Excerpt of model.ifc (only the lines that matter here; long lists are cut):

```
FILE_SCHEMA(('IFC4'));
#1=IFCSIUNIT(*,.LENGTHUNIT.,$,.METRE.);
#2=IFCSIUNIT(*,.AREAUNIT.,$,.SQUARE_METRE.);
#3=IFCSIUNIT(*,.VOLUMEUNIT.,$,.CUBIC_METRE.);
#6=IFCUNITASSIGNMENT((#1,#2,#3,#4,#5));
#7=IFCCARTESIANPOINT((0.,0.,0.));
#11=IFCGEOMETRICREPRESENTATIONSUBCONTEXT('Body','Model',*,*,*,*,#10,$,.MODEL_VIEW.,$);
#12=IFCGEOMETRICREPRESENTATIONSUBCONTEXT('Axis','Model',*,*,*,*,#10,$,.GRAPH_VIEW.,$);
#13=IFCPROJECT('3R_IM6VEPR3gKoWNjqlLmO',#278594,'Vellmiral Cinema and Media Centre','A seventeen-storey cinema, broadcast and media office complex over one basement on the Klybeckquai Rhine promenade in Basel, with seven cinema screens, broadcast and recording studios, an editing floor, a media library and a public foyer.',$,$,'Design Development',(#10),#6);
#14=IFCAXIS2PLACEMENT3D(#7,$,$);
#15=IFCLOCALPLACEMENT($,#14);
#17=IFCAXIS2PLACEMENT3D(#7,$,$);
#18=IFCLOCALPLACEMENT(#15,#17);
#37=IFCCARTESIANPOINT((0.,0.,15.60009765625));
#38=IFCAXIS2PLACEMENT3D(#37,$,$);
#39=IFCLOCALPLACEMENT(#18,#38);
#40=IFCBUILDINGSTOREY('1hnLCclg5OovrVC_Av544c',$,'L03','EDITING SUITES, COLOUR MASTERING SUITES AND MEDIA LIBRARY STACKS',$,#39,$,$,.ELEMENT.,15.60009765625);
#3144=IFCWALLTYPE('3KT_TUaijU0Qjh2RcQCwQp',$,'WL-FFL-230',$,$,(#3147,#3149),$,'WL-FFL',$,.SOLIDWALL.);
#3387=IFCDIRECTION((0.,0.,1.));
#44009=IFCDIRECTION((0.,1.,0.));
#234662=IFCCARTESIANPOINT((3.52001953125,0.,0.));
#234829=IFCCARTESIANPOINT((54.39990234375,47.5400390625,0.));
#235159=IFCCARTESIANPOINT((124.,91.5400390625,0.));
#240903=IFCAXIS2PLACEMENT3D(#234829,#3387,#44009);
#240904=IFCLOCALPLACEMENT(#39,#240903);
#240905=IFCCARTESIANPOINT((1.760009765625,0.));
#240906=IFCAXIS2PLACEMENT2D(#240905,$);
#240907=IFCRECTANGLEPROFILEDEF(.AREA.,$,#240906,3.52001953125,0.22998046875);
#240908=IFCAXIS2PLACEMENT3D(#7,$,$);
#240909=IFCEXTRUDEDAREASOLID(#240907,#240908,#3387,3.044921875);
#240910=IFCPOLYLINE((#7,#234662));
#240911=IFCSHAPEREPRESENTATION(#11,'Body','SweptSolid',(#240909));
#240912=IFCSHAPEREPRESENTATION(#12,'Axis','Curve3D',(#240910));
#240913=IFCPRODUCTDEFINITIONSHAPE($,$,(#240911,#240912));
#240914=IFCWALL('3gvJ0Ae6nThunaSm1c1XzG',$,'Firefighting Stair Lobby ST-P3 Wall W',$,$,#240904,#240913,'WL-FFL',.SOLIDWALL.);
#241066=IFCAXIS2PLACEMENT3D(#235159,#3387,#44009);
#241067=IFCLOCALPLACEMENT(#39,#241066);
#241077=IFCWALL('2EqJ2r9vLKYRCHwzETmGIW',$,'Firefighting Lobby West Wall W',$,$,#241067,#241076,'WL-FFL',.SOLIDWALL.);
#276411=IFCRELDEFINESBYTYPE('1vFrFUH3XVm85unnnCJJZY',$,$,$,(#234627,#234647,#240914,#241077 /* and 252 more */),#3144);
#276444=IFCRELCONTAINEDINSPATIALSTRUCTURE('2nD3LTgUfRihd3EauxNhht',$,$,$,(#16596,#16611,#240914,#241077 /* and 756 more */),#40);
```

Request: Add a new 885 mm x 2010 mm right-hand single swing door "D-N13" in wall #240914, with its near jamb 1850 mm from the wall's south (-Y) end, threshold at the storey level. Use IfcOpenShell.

```python
import numpy as np
import ifcopenshell
import ifcopenshell.api.feature
import ifcopenshell.api.geometry
import ifcopenshell.api.root
import ifcopenshell.api.spatial
import ifcopenshell.geom
import ifcopenshell.util.element
import ifcopenshell.util.placement
import ifcopenshell.util.representation
import ifcopenshell.util.shape
import ifcopenshell.util.unit

model = ifcopenshell.open("model.ifc")
unit_scale = ifcopenshell.util.unit.calculate_unit_scale(model)
settings = ifcopenshell.geom.settings()


def volume(element):
    """Net volume in cubic metres, openings subtracted."""
    shape = ifcopenshell.geom.create_shape(settings, element)
    return ifcopenshell.util.shape.get_volume(shape.geometry)


wall = model.by_guid("3gvJ0Ae6nThunaSm1c1XzG")
storey = ifcopenshell.util.element.get_container(wall, ifc_class="IfcBuildingStorey")
context = ifcopenshell.util.representation.get_context(model, "Model", "Body", "MODEL_VIEW")
before = volume(wall)

width, height, from_end, sill = 0.885, 2.01, 1.85, 0.0  # metres

# The wall runs along its own X axis, and the end named is its -X end.
wall_shape = ifcopenshell.geom.create_shape(settings, wall)
x, y, z = ifcopenshell.util.shape.get_vertices(wall_shape.geometry).T
start = x.min() + from_end
face, thickness = float(y.min()), float(y.max() - y.min())
wall_matrix = ifcopenshell.util.placement.get_local_placement(wall.ObjectPlacement)
level = ifcopenshell.util.placement.get_local_placement(storey.ObjectPlacement)[2, 3]


def in_wall(x, y):
    """Placement at x, y metres in the wall's axes, at sill height."""
    matrix = wall_matrix.copy()
    matrix[:, 3] = wall_matrix @ np.array([x / unit_scale, y / unit_scale, 0.0, 1.0])
    matrix[2, 3] = level + sill / unit_scale
    return matrix


# Opening: a box that overshoots both wall faces by 50 mm.
opening = ifcopenshell.api.root.create_entity(model, ifc_class="IfcOpeningElement", predefined_type="OPENING")
box = ifcopenshell.api.geometry.add_wall_representation(
    model, context=context, length=width, height=height, thickness=thickness + 0.1
)
ifcopenshell.api.geometry.assign_representation(model, product=opening, representation=box)
ifcopenshell.api.geometry.edit_object_placement(model, product=opening, matrix=in_wall(start, face - 0.05), is_si=False)
ifcopenshell.api.feature.add_feature(model, feature=opening, element=wall)

door = ifcopenshell.api.root.create_entity(model, ifc_class="IfcDoor", name="D-N13", predefined_type="DOOR")
door.OverallWidth, door.OverallHeight = width / unit_scale, height / unit_scale
door.OperationType = "SINGLE_SWING_RIGHT"
body = ifcopenshell.api.geometry.add_door_representation(
    model,
    context=context,
    overall_width=door.OverallWidth,
    overall_height=door.OverallHeight,
    operation_type="SINGLE_SWING_RIGHT",
    lining_properties={"LiningDepth": thickness / unit_scale, "ThresholdDepth": thickness / unit_scale},
)
ifcopenshell.api.geometry.assign_representation(model, product=door, representation=body)
ifcopenshell.api.spatial.assign_container(model, products=[door], relating_structure=storey)
ifcopenshell.api.feature.add_filling(model, opening=opening, element=door)

# The lining spans the wall, so the door starts at the wall face.
ifcopenshell.api.geometry.edit_object_placement(model, product=door, matrix=in_wall(start, face), is_si=False)

after = volume(wall)

print(f"wall volume {before:.3f} -> {after:.3f} m3")

model.write("model_edited.ifc")
```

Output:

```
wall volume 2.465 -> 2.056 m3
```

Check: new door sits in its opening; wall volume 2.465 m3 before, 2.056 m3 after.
